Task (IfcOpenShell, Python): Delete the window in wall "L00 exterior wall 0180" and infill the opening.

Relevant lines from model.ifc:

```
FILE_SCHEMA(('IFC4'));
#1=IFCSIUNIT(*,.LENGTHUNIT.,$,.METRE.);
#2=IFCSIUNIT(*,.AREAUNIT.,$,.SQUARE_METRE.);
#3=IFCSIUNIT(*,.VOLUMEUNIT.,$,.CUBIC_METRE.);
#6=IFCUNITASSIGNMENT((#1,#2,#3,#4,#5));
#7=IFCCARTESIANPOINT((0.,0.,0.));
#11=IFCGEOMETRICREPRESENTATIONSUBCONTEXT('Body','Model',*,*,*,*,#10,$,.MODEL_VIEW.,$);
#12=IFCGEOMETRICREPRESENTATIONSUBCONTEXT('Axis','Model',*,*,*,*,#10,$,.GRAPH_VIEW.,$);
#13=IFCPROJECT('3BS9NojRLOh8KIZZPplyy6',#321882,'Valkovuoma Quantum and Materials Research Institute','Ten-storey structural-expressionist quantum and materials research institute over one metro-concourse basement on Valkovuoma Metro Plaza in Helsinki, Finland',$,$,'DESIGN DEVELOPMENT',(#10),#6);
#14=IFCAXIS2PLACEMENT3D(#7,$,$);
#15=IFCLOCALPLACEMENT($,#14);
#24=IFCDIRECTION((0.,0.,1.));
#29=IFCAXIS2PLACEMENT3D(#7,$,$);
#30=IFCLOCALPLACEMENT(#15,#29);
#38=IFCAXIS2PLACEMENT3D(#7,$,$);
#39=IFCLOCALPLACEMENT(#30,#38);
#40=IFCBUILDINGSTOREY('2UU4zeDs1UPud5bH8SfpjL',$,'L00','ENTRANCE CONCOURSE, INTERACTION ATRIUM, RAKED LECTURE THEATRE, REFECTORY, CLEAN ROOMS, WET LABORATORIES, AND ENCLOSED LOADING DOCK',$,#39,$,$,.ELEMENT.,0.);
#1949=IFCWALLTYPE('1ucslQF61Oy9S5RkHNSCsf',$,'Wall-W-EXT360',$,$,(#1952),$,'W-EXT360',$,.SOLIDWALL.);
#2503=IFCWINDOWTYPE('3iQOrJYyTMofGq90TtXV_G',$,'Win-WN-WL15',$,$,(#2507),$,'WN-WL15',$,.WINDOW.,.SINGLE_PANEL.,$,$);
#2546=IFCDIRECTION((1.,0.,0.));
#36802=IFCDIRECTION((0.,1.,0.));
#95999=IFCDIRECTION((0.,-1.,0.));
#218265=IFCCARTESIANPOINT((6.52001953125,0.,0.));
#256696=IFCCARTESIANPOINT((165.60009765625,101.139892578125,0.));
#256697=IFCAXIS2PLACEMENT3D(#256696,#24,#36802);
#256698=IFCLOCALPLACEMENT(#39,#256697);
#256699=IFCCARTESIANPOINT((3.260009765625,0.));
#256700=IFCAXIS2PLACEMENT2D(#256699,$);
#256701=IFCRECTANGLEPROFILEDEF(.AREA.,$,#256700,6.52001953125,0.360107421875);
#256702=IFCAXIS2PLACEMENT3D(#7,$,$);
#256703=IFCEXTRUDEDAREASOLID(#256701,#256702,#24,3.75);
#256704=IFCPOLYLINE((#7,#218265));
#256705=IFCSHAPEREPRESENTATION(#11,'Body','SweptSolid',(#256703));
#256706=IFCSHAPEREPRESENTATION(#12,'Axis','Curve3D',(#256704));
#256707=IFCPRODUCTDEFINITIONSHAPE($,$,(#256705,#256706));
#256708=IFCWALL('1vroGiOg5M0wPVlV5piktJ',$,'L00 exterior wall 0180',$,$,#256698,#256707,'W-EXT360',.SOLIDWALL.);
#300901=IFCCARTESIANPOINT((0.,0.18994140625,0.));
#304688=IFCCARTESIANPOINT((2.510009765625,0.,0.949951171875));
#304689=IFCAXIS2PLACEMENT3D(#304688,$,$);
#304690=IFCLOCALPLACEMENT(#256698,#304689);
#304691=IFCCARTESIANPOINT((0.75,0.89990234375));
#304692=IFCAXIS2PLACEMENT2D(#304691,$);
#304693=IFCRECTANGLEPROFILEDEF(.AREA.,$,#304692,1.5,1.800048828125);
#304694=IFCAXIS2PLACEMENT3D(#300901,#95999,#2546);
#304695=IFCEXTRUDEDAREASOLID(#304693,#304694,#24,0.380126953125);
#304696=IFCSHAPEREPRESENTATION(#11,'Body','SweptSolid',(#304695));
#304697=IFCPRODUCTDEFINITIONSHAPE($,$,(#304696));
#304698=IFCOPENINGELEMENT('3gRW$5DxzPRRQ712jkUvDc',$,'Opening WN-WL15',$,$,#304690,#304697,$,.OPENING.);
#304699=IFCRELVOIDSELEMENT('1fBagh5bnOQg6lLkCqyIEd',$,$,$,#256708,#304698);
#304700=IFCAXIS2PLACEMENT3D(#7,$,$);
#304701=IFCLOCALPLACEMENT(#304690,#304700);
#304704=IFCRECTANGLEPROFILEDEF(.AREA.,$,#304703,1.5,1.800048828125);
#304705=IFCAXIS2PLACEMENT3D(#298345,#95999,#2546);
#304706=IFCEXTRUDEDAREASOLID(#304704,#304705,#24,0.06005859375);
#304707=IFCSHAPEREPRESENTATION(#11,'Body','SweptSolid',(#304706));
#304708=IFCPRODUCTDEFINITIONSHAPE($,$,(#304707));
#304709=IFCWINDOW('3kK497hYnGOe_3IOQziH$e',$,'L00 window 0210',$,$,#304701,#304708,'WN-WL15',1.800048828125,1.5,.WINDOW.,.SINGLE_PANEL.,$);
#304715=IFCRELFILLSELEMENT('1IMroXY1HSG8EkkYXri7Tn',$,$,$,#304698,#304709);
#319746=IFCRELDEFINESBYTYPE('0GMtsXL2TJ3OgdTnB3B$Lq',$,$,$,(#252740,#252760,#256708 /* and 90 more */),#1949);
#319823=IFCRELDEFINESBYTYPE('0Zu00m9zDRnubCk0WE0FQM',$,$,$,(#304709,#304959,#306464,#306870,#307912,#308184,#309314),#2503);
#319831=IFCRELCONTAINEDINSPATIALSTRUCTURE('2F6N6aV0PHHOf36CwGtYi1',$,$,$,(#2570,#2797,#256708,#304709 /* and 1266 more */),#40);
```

```python
import ifcopenshell
import ifcopenshell.api.feature
import ifcopenshell.api.root
import ifcopenshell.geom
import ifcopenshell.util.shape

model = ifcopenshell.open("model.ifc")
settings = ifcopenshell.geom.settings()


def volume(element):
    """Net volume in cubic metres, openings subtracted."""
    shape = ifcopenshell.geom.create_shape(settings, element)
    return ifcopenshell.util.shape.get_volume(shape.geometry)


window = model.by_guid("3kK497hYnGOe_3IOQziH$e")
opening = window.FillsVoids[0].RelatingOpeningElement
wall = opening.VoidsElements[0].RelatingBuildingElement
before = volume(wall)

ifcopenshell.api.root.remove_product(model, product=window)
ifcopenshell.api.feature.remove_feature(model, feature=opening)

after = volume(wall)

print(f"wall volume {before:.3f} -> {after:.3f} m3")

model.write("model_edited.ifc")
```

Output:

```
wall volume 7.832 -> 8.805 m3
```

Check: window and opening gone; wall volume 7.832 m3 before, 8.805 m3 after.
